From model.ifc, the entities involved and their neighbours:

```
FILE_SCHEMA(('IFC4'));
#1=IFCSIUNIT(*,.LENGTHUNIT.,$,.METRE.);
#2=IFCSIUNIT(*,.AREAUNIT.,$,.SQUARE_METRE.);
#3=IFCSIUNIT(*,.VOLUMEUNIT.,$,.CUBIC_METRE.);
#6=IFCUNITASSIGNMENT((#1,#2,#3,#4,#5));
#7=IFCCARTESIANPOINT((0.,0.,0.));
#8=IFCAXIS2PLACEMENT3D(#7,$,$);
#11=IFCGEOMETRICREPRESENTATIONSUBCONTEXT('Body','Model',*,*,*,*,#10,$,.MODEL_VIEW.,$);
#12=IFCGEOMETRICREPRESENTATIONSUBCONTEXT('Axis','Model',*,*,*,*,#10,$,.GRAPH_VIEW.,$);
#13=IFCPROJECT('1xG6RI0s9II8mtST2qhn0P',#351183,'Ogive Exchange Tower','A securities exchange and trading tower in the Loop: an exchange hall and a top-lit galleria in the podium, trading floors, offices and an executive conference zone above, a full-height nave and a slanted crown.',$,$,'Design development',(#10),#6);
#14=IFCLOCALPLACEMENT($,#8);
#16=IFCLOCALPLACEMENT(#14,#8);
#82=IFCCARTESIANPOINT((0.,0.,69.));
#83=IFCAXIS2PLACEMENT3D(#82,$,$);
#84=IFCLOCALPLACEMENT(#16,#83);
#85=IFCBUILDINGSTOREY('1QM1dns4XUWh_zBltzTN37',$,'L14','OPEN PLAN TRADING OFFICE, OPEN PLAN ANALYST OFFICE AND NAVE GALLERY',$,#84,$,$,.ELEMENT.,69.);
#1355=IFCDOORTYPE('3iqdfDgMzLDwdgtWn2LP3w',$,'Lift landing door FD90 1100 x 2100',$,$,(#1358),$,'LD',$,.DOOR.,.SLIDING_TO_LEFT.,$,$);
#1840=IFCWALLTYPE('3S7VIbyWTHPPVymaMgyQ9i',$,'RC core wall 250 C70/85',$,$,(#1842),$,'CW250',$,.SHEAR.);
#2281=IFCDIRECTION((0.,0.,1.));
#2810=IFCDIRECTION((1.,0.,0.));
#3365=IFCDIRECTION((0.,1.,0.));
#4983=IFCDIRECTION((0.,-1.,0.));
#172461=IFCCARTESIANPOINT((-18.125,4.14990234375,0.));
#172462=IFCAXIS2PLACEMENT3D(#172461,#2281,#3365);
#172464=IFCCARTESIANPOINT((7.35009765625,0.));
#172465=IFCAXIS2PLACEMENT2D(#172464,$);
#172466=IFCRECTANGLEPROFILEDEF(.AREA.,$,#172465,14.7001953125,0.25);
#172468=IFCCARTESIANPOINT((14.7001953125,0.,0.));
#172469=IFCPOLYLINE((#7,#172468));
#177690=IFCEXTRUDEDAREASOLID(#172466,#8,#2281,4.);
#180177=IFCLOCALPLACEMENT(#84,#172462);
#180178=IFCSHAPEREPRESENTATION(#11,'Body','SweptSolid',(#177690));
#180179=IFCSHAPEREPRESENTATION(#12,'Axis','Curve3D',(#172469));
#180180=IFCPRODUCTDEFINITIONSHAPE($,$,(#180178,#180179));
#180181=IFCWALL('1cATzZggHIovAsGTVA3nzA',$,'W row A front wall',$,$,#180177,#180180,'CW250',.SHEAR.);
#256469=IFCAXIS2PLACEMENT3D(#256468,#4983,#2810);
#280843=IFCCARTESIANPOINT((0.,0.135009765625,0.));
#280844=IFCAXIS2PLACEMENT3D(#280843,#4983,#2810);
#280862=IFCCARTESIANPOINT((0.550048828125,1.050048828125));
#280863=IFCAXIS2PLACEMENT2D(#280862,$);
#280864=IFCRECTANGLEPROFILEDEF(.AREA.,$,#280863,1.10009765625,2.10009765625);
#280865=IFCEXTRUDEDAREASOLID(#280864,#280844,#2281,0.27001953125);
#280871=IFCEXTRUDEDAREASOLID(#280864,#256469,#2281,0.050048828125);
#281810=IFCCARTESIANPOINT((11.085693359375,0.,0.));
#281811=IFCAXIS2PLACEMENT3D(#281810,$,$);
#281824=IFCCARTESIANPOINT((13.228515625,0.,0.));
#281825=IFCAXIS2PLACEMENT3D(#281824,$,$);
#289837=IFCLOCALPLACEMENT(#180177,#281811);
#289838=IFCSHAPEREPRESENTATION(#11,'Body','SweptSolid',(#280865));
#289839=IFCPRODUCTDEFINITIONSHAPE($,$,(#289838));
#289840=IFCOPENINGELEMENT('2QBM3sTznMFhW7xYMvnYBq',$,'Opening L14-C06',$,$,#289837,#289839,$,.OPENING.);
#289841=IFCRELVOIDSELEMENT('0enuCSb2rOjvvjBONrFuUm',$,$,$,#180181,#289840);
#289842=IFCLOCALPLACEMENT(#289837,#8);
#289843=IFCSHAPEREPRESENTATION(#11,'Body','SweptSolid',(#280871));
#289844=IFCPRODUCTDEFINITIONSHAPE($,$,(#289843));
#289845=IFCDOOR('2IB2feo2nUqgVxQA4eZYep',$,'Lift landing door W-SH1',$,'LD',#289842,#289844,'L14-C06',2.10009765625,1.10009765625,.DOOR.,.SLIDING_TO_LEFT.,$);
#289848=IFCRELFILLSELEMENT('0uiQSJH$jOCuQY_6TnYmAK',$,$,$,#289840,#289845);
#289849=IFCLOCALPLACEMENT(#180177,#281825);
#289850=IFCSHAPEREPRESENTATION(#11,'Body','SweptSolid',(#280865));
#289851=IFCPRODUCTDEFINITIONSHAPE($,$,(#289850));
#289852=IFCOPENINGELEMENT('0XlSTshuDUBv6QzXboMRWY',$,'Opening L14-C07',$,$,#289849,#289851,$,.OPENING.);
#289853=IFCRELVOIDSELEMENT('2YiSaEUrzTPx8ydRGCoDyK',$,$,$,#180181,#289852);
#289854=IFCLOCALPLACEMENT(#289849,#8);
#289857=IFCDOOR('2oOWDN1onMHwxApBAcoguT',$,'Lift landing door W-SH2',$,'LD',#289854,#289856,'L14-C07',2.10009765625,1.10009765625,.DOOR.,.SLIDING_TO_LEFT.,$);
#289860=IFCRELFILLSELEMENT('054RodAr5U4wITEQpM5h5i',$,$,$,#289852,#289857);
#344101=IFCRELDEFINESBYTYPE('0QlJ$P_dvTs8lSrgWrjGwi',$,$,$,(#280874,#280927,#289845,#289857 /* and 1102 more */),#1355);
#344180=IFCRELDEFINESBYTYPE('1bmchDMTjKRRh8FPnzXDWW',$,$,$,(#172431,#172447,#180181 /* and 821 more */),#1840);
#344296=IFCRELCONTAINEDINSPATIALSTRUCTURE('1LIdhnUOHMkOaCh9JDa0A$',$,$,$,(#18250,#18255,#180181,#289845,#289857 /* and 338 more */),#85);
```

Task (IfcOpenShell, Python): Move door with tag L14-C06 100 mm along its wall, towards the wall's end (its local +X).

```python
import ifcopenshell
import ifcopenshell.api.geometry
import ifcopenshell.util.placement
import ifcopenshell.util.unit

model = ifcopenshell.open("model.ifc")
unit_scale = ifcopenshell.util.unit.calculate_unit_scale(model)

door = model.by_id(289845)
opening = door.FillsVoids[0].RelatingOpeningElement
wall = opening.VoidsElements[0].RelatingBuildingElement

wall_matrix = ifcopenshell.util.placement.get_local_placement(wall.ObjectPlacement)
shift = wall_matrix[:3, 0] * 0.1 / unit_scale
before = ifcopenshell.util.placement.get_local_placement(door.ObjectPlacement)[:3, 3].copy()

# The door is placed relative to its opening, so it follows when the opening moves.
matrix = ifcopenshell.util.placement.get_local_placement(opening.ObjectPlacement)
matrix[:3, 3] += shift
ifcopenshell.api.geometry.edit_object_placement(
    model, product=opening, matrix=matrix, is_si=False, should_transform_children=True
)

after = ifcopenshell.util.placement.get_local_placement(door.ObjectPlacement)[:3, 3]
print("door moved by", (after - before).round(3) + 0.0)

model.write("model_updated.ifc")
```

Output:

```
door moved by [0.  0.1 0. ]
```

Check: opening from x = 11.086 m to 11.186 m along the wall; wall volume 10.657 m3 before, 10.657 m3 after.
